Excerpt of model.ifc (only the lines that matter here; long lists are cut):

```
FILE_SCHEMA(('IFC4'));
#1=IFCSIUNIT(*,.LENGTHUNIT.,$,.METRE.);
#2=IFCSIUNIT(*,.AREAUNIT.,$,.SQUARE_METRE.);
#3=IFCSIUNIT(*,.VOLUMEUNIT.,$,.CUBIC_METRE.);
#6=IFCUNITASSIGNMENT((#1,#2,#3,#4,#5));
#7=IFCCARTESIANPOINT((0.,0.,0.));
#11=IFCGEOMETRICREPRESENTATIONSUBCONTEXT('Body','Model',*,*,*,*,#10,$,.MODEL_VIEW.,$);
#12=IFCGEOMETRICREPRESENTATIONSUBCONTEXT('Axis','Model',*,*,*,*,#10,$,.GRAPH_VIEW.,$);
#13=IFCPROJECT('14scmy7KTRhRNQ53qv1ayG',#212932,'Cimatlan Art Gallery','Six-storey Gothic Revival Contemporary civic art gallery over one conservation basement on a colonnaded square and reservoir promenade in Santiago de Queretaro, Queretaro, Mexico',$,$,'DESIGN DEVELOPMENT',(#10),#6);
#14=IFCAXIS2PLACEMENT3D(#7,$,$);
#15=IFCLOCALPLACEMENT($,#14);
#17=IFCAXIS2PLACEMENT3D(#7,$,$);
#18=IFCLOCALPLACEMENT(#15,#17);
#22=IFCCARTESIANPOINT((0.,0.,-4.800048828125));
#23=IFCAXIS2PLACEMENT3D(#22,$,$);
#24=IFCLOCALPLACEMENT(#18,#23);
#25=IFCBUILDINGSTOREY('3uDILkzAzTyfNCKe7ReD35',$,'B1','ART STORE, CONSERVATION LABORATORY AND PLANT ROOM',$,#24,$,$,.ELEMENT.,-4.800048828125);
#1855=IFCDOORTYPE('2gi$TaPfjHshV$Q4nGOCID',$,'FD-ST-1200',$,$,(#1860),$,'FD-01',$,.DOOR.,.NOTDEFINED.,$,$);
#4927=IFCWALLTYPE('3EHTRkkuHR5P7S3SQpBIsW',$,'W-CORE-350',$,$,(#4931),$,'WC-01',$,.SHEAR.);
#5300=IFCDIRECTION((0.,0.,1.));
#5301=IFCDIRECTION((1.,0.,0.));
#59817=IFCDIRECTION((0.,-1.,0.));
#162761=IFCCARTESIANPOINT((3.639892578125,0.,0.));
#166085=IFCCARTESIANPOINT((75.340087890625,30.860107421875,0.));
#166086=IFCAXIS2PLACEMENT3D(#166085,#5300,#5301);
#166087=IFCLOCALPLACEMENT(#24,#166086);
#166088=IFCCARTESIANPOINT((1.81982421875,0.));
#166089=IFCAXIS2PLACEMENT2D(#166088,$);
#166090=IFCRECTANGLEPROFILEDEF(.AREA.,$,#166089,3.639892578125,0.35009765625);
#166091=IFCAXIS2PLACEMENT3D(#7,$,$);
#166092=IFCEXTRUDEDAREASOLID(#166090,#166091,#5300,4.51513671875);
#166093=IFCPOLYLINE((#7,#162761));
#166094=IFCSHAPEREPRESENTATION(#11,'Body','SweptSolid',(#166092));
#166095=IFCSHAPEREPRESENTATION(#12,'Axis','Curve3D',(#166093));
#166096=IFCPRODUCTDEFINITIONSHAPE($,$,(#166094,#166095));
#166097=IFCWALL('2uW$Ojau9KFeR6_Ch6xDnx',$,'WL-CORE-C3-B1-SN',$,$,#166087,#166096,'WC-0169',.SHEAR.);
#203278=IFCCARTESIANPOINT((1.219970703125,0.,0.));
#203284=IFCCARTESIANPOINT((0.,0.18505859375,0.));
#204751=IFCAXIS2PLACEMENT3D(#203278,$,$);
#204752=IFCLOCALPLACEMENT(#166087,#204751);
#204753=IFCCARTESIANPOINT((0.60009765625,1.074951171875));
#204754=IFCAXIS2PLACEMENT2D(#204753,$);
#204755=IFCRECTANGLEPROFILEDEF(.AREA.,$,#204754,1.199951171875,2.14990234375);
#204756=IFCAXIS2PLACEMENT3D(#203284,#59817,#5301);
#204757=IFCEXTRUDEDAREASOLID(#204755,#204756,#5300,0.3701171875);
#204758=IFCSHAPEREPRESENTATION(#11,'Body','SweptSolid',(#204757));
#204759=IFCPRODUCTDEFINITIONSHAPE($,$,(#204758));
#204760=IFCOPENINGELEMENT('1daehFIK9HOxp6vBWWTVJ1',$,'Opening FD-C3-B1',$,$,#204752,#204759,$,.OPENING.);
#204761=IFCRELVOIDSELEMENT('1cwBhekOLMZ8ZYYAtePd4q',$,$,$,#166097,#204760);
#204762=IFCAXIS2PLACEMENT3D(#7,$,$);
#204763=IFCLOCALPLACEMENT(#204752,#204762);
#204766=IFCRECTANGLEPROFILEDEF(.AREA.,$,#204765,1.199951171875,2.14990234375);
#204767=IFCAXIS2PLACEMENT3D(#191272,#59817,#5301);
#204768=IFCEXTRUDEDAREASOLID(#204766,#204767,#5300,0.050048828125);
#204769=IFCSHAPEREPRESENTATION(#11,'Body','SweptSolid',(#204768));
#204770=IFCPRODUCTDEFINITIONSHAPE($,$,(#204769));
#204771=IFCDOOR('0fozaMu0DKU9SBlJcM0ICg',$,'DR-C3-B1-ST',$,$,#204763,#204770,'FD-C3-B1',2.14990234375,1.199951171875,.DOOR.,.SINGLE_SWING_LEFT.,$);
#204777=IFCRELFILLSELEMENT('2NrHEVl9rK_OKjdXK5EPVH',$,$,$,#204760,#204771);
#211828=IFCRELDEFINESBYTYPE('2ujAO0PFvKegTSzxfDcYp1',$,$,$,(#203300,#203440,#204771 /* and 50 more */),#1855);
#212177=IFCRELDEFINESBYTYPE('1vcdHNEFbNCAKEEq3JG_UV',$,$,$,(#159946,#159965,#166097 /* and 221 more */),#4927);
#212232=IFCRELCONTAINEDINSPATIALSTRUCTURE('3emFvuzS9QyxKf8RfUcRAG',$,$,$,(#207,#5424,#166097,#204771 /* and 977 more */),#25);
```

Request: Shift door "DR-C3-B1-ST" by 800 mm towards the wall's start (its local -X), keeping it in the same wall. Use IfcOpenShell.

```python
import ifcopenshell
import ifcopenshell.api.geometry
import ifcopenshell.util.placement

model = ifcopenshell.open("model.ifc")

door = model.by_guid("0fozaMu0DKU9SBlJcM0ICg")
opening = door.FillsVoids[0].RelatingOpeningElement
wall = opening.VoidsElements[0].RelatingBuildingElement

wall_matrix = ifcopenshell.util.placement.get_local_placement(wall.ObjectPlacement)
shift = wall_matrix[:3, 0] * -0.8
before = ifcopenshell.util.placement.get_local_placement(door.ObjectPlacement)[:3, 3].copy()

# The door is placed relative to its opening, so it follows when the opening moves.
matrix = ifcopenshell.util.placement.get_local_placement(opening.ObjectPlacement)
matrix[:3, 3] += shift
ifcopenshell.api.geometry.edit_object_placement(
    model, product=opening, matrix=matrix, is_si=False, should_transform_children=True
)

after = ifcopenshell.util.placement.get_local_placement(door.ObjectPlacement)[:3, 3]
print("door moved by", (after - before).round(3) + 0.0)

model.write("model_v2.ifc")
```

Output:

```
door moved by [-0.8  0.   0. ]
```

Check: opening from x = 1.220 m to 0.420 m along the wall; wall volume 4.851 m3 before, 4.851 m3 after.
